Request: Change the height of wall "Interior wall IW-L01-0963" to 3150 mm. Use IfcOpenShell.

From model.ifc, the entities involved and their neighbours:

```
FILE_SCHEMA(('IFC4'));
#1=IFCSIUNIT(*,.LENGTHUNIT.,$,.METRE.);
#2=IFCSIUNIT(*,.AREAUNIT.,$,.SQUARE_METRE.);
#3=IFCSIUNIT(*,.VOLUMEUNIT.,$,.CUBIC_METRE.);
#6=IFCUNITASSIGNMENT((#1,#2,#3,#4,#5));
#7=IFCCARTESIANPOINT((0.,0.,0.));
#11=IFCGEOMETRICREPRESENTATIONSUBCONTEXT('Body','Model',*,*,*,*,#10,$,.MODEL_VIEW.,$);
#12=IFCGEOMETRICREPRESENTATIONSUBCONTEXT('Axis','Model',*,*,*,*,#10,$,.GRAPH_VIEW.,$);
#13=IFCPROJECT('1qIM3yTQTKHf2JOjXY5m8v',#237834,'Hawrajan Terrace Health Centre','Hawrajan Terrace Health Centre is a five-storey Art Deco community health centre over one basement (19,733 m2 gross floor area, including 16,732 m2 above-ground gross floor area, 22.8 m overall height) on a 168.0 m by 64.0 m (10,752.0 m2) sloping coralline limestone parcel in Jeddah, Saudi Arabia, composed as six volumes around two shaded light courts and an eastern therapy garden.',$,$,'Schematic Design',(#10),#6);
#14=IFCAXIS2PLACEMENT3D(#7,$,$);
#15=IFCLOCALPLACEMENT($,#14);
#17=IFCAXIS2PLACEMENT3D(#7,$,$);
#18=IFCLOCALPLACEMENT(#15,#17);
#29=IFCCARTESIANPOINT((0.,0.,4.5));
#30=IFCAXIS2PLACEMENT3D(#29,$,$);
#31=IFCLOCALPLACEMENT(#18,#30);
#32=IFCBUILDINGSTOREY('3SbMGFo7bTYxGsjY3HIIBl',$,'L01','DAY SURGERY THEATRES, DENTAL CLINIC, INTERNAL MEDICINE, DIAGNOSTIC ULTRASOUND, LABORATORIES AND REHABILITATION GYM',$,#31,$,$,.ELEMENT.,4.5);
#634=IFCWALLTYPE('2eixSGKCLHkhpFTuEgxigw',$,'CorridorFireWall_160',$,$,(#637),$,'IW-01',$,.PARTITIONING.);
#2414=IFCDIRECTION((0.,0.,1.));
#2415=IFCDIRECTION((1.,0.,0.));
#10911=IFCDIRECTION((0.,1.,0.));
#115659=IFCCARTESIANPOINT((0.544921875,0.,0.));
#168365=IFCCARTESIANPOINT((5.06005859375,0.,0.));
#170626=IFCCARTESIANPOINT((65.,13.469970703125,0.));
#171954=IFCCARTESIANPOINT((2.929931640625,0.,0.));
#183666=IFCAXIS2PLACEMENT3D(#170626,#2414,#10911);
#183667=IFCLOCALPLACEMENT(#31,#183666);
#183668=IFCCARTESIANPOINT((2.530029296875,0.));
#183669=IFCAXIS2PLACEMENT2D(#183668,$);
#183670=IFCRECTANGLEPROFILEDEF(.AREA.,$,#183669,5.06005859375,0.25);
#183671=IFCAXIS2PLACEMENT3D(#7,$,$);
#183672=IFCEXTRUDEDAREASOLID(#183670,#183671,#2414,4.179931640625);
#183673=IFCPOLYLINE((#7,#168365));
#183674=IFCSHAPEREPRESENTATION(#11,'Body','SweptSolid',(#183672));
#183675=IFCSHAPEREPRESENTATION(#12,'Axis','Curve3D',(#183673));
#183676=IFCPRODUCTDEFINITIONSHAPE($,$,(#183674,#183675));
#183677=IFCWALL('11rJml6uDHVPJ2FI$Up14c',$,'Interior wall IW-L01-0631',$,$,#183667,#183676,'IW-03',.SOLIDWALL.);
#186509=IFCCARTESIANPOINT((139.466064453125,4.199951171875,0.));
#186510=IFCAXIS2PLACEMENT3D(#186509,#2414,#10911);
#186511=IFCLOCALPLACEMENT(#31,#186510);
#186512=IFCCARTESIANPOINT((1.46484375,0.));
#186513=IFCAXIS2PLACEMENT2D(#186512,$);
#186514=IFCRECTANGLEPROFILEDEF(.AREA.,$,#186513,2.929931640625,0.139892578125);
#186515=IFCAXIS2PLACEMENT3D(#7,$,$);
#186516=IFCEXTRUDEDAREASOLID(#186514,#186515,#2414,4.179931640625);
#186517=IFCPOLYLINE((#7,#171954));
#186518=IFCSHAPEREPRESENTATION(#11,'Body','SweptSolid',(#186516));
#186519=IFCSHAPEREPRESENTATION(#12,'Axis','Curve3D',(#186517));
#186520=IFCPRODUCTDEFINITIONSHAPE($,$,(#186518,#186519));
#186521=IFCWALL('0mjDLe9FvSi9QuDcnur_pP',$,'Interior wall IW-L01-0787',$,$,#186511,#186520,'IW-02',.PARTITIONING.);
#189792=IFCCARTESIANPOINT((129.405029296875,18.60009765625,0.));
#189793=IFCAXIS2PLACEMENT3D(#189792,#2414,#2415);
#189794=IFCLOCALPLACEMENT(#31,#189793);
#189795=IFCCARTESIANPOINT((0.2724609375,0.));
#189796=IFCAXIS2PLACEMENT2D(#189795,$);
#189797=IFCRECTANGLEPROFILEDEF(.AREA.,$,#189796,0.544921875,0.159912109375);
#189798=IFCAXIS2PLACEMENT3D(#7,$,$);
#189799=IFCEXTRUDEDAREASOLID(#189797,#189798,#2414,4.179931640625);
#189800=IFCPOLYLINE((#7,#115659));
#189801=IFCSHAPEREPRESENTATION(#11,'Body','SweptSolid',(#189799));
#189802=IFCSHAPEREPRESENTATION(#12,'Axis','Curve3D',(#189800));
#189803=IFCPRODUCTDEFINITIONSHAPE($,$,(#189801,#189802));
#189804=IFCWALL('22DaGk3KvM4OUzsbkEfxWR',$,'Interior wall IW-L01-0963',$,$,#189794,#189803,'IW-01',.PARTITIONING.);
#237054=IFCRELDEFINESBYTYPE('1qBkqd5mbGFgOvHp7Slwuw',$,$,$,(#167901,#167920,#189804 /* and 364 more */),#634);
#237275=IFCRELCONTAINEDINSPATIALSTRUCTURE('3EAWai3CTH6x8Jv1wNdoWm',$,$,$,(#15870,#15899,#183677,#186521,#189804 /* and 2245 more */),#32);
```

```python
import ifcopenshell
import ifcopenshell.geom
import ifcopenshell.util.representation
import ifcopenshell.util.shape

model = ifcopenshell.open("model.ifc")
settings = ifcopenshell.geom.settings()


def volume(element):
    """Net volume in cubic metres, openings subtracted."""
    shape = ifcopenshell.geom.create_shape(settings, element)
    return ifcopenshell.util.shape.get_volume(shape.geometry)


wall = model.by_guid("22DaGk3KvM4OUzsbkEfxWR")
before = volume(wall)

body = ifcopenshell.util.representation.get_representation(wall, "Model", "Body")
solid = body.Items[0]
old_height = solid.Depth
solid.Depth = 3.15
after = volume(wall)

print(f"height {old_height:g} -> {solid.Depth:g}, volume {before:.3f} -> {after:.3f} m3")

model.write("model_rev.ifc")
```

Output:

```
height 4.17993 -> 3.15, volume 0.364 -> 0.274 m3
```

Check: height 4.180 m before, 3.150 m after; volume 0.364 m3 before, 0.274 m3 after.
